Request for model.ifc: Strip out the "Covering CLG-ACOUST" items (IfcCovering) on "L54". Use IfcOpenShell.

First a look at what the model holds.

```python
import ifcopenshell
import ifcopenshell.util.element

model = ifcopenshell.open("model.ifc")
print(model.schema)
storey = next(s for s in model.by_type("IfcBuildingStorey") if s.Name == "L54")
coverings = [e for e in ifcopenshell.util.element.get_decomposition(storey) if e.is_a("IfcCovering")]
seen = {}
for e in coverings:
    element_type = ifcopenshell.util.element.get_type(e)
    name = element_type.Name if element_type not in (None, e) else None
    seen[name] = seen.get(name, 0) + 1
for name, count in sorted(seen.items(), key=str):
    print(count, "x", name)
```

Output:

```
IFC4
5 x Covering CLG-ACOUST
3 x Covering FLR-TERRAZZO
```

```python
import ifcopenshell
import ifcopenshell.api.root
import ifcopenshell.util.element

model = ifcopenshell.open("model.ifc")

storey = next(s for s in model.by_type("IfcBuildingStorey") if s.Name == "L54")
coverings = [e for e in ifcopenshell.util.element.get_decomposition(storey) if e.is_a("IfcCovering")]
targets = [e for e in coverings if (t := ifcopenshell.util.element.get_type(e)) not in (None, e) and t.Name == "Covering CLG-ACOUST"]

for e in targets:
    ifcopenshell.api.root.remove_product(model, product=e)
print(len(targets), "removed")

model.write("model-out.ifc")
```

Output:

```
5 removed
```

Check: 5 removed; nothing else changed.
